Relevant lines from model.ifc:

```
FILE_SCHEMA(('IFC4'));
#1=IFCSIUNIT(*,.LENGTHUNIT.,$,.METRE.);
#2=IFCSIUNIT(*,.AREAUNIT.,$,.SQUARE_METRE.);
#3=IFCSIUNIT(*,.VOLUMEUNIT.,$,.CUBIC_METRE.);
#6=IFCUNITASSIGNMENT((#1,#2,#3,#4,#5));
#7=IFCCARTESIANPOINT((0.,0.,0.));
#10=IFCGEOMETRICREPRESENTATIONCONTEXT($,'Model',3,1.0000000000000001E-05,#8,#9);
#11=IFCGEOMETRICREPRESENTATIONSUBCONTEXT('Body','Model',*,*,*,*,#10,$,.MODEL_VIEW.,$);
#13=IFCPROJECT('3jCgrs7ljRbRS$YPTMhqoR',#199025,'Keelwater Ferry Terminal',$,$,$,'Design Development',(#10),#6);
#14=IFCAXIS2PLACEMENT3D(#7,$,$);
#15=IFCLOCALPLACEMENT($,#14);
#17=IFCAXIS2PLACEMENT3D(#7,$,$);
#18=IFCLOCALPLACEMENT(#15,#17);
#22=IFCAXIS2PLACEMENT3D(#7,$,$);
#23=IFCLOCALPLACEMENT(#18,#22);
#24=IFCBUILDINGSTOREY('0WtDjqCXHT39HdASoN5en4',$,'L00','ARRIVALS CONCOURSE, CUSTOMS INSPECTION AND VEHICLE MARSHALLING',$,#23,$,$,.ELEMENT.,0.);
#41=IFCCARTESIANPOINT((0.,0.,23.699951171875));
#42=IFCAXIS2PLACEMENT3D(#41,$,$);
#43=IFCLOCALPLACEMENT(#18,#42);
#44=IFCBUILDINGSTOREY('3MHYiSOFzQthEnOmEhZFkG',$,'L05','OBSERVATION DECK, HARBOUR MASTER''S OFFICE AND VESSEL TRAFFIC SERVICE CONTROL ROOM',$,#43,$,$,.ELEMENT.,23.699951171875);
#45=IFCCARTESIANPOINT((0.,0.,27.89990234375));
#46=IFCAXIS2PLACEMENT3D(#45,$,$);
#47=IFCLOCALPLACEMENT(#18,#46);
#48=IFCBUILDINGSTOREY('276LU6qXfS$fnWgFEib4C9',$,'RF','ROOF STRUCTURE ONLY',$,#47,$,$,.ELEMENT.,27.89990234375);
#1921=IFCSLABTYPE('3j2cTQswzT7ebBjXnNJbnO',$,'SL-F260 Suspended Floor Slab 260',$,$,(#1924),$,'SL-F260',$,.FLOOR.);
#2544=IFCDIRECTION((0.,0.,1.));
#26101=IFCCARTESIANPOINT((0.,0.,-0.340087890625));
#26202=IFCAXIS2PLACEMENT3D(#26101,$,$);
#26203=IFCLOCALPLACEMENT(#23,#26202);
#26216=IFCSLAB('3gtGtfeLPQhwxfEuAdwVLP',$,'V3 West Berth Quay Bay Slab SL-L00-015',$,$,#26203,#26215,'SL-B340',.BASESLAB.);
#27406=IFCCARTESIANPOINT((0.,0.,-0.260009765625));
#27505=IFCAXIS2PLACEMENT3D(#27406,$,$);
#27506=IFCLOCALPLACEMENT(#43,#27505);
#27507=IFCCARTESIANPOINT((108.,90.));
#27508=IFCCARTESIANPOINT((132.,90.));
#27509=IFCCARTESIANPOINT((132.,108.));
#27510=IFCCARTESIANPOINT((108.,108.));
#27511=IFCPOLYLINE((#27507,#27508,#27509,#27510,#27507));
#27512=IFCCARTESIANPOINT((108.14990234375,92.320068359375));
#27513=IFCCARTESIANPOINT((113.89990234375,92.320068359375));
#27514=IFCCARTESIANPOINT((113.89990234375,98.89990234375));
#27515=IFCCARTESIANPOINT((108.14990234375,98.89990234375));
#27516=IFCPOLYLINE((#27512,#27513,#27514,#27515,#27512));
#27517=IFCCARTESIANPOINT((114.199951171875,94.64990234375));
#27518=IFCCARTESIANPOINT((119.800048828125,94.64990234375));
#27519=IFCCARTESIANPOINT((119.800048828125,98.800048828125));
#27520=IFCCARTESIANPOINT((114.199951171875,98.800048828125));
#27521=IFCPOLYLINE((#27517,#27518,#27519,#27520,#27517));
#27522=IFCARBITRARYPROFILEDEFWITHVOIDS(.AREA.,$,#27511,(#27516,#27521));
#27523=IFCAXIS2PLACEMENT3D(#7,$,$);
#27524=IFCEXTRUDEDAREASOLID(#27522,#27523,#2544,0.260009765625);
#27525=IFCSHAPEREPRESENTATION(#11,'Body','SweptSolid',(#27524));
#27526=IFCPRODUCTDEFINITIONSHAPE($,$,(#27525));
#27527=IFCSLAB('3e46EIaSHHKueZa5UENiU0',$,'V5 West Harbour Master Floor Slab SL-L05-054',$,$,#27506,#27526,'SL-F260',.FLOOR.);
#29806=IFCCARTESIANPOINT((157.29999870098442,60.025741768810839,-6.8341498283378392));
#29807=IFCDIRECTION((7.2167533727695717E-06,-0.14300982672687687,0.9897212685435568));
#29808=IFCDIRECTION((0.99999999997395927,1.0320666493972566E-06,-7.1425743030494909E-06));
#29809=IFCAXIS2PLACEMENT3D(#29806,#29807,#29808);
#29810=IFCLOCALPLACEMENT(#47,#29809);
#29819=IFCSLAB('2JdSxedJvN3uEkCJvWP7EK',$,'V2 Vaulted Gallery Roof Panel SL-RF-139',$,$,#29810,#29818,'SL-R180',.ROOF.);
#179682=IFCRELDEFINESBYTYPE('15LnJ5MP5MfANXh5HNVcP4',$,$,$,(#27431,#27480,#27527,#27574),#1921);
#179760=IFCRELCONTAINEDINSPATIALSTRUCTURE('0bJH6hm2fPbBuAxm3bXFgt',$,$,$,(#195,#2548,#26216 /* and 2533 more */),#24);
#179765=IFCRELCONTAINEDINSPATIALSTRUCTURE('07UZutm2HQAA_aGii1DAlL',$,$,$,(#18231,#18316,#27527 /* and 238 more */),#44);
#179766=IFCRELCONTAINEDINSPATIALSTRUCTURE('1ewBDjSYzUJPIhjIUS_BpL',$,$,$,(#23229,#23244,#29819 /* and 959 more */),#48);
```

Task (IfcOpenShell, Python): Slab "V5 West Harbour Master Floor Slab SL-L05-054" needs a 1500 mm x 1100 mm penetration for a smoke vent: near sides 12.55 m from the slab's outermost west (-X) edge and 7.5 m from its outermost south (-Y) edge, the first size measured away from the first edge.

```python
import numpy as np
import ifcopenshell
import ifcopenshell.api.feature
import ifcopenshell.api.geometry
import ifcopenshell.api.root
import ifcopenshell.geom
import ifcopenshell.util.placement
import ifcopenshell.util.representation
import ifcopenshell.util.shape
import ifcopenshell.util.unit

model = ifcopenshell.open("model.ifc")
unit_scale = ifcopenshell.util.unit.calculate_unit_scale(model)
settings = ifcopenshell.geom.settings()


def volume(element):
    """Net volume in cubic metres, openings subtracted."""
    shape = ifcopenshell.geom.create_shape(settings, element)
    return ifcopenshell.util.shape.get_volume(shape.geometry)


slab = model.by_guid("3e46EIaSHHKueZa5UENiU0")
before = volume(slab)

# Extent in the slab's own axes, in metres. The edges named are its -X and -Y sides.
slab_shape = ifcopenshell.geom.create_shape(settings, slab)
vertices = ifcopenshell.util.shape.get_vertices(slab_shape.geometry)
x_min, y_min, bottom = vertices.min(axis=0)
top = vertices[:, 2].max()

opening = ifcopenshell.api.root.create_entity(model, ifc_class="IfcOpeningElement", name="Smoke vent opening", predefined_type="OPENING")
context = ifcopenshell.util.representation.get_context(model, "Model", "Body", "MODEL_VIEW")
width, depth = 1.5, 1.1
outline = [(0.0, 0.0), (width, 0.0), (width, depth), (0.0, depth), (0.0, 0.0)]
# Overshoot both faces by 50 mm so the cut is clean.
shape = ifcopenshell.api.geometry.add_slab_representation(
    model, context=context, depth=top - bottom + 0.1, polyline=outline
)
ifcopenshell.api.geometry.assign_representation(model, product=opening, representation=shape)

matrix = ifcopenshell.util.placement.get_local_placement(slab.ObjectPlacement)
matrix[:, 3] = matrix @ np.append(np.array([x_min + 12.55, y_min + 7.5, bottom - 0.05]) / unit_scale, 1.0)
ifcopenshell.api.geometry.edit_object_placement(model, product=opening, matrix=matrix, is_si=False)
ifcopenshell.api.feature.add_feature(model, feature=opening, element=slab)

after = volume(slab)

print(f"slab volume {before:.3f} -> {after:.3f} m3")

model.write("model_edited.ifc")
```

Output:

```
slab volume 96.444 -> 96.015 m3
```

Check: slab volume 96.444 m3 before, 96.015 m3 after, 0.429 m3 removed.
